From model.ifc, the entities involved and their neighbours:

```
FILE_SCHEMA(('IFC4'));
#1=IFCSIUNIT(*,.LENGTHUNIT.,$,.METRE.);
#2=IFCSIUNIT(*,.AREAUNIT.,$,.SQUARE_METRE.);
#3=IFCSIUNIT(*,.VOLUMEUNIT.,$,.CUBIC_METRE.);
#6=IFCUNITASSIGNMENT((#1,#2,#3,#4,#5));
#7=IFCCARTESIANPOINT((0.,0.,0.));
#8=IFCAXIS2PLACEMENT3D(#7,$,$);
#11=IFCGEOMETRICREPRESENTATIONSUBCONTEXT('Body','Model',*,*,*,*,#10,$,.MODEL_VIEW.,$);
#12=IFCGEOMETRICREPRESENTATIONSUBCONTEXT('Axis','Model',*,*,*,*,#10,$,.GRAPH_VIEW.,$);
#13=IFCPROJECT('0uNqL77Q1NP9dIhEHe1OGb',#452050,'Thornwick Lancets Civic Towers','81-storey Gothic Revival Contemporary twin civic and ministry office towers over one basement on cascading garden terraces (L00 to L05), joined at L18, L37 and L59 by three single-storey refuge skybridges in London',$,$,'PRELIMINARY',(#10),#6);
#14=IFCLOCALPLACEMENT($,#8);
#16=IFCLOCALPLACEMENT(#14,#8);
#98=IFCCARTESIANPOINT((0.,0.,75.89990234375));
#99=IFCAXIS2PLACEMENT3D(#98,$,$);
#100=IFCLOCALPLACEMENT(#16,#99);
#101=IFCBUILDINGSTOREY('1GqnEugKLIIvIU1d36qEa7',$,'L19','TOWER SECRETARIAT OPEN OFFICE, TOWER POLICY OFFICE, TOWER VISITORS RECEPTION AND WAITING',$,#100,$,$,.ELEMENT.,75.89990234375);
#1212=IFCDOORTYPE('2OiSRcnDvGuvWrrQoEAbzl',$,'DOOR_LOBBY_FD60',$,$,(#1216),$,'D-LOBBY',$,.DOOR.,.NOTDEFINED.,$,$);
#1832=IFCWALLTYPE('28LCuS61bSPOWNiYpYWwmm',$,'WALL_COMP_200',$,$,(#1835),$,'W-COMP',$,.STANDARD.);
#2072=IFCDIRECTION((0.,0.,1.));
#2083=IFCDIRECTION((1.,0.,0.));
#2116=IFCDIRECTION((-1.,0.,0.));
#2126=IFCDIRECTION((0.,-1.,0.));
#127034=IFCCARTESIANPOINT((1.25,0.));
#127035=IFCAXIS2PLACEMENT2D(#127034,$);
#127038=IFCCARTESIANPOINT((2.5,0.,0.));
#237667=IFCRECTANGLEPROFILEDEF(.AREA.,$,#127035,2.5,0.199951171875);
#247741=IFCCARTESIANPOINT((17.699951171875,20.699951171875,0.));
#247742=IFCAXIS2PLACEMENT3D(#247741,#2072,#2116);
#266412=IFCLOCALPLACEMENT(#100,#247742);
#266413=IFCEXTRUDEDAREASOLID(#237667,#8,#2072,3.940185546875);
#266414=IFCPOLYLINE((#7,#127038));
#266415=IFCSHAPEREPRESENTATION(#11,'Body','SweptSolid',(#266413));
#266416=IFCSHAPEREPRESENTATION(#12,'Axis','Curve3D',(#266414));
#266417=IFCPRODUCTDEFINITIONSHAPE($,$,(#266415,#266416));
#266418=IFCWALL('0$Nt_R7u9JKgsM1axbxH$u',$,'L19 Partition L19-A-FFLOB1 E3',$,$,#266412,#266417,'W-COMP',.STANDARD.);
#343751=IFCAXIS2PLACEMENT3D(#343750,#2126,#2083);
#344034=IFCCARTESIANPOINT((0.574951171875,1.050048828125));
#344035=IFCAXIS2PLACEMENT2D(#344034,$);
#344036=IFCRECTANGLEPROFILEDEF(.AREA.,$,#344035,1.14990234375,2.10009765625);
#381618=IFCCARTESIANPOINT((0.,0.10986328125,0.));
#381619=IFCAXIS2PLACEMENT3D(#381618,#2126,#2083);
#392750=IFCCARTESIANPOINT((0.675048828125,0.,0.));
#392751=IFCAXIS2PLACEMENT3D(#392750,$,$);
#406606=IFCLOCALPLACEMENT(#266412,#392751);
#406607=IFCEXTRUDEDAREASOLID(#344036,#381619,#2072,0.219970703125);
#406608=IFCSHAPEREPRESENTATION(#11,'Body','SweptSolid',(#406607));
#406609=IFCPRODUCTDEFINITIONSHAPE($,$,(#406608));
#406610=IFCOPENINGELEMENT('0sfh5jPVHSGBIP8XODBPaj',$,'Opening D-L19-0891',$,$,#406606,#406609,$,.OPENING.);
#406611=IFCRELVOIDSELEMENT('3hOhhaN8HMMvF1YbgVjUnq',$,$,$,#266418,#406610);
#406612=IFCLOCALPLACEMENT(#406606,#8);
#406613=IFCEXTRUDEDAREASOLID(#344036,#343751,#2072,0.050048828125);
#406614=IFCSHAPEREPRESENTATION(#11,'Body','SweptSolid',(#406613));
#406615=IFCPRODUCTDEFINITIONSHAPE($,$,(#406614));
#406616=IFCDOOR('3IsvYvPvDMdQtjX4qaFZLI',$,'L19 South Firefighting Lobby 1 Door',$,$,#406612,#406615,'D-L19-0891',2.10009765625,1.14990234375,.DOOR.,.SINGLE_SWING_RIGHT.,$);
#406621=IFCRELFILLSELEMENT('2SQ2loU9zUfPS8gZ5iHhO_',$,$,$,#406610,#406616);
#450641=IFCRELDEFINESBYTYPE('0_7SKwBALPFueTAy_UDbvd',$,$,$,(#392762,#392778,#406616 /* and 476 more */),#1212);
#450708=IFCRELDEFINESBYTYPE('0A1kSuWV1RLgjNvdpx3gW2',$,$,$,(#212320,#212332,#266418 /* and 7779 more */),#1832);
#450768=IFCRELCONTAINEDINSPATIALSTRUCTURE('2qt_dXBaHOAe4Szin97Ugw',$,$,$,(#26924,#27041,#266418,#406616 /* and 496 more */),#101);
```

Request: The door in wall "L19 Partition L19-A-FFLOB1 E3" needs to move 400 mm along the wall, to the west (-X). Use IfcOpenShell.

```python
import ifcopenshell
import ifcopenshell.api.geometry
import ifcopenshell.util.placement
import ifcopenshell.util.unit

model = ifcopenshell.open("model.ifc")
unit_scale = ifcopenshell.util.unit.calculate_unit_scale(model)

door = model.by_id(406616)
opening = door.FillsVoids[0].RelatingOpeningElement
wall = opening.VoidsElements[0].RelatingBuildingElement

wall_matrix = ifcopenshell.util.placement.get_local_placement(wall.ObjectPlacement)
shift = wall_matrix[:3, 0] * 0.4 / unit_scale
before = ifcopenshell.util.placement.get_local_placement(door.ObjectPlacement)[:3, 3].copy()

# The door is placed relative to its opening, so it follows when the opening moves.
matrix = ifcopenshell.util.placement.get_local_placement(opening.ObjectPlacement)
matrix[:3, 3] += shift
ifcopenshell.api.geometry.edit_object_placement(
    model, product=opening, matrix=matrix, is_si=False, should_transform_children=True
)

after = ifcopenshell.util.placement.get_local_placement(door.ObjectPlacement)[:3, 3]
print("door moved by", (after - before).round(3) + 0.0)

model.write("model_rev.ifc")
```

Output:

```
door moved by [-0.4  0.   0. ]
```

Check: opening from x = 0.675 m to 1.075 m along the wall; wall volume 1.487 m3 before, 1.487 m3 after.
